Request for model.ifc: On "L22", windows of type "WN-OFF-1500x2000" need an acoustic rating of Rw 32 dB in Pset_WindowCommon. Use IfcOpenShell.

First a look at what the model holds.

```python
import ifcopenshell
import ifcopenshell.util.element

model = ifcopenshell.open("model.ifc")
print(model.schema)
storey = next(s for s in model.by_type("IfcBuildingStorey") if s.Name == "L22")
windows = [e for e in ifcopenshell.util.element.get_decomposition(storey) if e.is_a("IfcWindow")]
seen = {}
for e in windows:
    element_type = ifcopenshell.util.element.get_type(e)
    key = (element_type.Name if element_type != e and element_type else None, ifcopenshell.util.element.get_pset(e, "Pset_WindowCommon", "AcousticRating"))
    seen[key] = seen.get(key, 0) + 1
for (name, value), count in sorted(seen.items(), key=str):
    print(count, "x", name, "|", value)
```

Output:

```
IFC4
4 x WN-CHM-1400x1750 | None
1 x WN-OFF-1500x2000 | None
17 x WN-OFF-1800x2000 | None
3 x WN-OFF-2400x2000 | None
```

```python
import ifcopenshell
import ifcopenshell.api.pset
import ifcopenshell.util.element

model = ifcopenshell.open("model.ifc")

storey = next(s for s in model.by_type("IfcBuildingStorey") if s.Name == "L22")
windows = [e for e in ifcopenshell.util.element.get_decomposition(storey) if e.is_a("IfcWindow")]

count = 0
for e in windows:
    element_type = ifcopenshell.util.element.get_type(e)
    if element_type in (None, e) or element_type.Name != "WN-OFF-1500x2000":
        continue
    # add_pset returns the element's existing set when there is one.
    pset = ifcopenshell.api.pset.add_pset(model, product=e, name="Pset_WindowCommon")
    ifcopenshell.api.pset.edit_pset(model, pset=pset, properties={"AcousticRating": "Rw 32 dB"})
    count += 1

print(count, "windows updated")

model.write("model_edited.ifc")
```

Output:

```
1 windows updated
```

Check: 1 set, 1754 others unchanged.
